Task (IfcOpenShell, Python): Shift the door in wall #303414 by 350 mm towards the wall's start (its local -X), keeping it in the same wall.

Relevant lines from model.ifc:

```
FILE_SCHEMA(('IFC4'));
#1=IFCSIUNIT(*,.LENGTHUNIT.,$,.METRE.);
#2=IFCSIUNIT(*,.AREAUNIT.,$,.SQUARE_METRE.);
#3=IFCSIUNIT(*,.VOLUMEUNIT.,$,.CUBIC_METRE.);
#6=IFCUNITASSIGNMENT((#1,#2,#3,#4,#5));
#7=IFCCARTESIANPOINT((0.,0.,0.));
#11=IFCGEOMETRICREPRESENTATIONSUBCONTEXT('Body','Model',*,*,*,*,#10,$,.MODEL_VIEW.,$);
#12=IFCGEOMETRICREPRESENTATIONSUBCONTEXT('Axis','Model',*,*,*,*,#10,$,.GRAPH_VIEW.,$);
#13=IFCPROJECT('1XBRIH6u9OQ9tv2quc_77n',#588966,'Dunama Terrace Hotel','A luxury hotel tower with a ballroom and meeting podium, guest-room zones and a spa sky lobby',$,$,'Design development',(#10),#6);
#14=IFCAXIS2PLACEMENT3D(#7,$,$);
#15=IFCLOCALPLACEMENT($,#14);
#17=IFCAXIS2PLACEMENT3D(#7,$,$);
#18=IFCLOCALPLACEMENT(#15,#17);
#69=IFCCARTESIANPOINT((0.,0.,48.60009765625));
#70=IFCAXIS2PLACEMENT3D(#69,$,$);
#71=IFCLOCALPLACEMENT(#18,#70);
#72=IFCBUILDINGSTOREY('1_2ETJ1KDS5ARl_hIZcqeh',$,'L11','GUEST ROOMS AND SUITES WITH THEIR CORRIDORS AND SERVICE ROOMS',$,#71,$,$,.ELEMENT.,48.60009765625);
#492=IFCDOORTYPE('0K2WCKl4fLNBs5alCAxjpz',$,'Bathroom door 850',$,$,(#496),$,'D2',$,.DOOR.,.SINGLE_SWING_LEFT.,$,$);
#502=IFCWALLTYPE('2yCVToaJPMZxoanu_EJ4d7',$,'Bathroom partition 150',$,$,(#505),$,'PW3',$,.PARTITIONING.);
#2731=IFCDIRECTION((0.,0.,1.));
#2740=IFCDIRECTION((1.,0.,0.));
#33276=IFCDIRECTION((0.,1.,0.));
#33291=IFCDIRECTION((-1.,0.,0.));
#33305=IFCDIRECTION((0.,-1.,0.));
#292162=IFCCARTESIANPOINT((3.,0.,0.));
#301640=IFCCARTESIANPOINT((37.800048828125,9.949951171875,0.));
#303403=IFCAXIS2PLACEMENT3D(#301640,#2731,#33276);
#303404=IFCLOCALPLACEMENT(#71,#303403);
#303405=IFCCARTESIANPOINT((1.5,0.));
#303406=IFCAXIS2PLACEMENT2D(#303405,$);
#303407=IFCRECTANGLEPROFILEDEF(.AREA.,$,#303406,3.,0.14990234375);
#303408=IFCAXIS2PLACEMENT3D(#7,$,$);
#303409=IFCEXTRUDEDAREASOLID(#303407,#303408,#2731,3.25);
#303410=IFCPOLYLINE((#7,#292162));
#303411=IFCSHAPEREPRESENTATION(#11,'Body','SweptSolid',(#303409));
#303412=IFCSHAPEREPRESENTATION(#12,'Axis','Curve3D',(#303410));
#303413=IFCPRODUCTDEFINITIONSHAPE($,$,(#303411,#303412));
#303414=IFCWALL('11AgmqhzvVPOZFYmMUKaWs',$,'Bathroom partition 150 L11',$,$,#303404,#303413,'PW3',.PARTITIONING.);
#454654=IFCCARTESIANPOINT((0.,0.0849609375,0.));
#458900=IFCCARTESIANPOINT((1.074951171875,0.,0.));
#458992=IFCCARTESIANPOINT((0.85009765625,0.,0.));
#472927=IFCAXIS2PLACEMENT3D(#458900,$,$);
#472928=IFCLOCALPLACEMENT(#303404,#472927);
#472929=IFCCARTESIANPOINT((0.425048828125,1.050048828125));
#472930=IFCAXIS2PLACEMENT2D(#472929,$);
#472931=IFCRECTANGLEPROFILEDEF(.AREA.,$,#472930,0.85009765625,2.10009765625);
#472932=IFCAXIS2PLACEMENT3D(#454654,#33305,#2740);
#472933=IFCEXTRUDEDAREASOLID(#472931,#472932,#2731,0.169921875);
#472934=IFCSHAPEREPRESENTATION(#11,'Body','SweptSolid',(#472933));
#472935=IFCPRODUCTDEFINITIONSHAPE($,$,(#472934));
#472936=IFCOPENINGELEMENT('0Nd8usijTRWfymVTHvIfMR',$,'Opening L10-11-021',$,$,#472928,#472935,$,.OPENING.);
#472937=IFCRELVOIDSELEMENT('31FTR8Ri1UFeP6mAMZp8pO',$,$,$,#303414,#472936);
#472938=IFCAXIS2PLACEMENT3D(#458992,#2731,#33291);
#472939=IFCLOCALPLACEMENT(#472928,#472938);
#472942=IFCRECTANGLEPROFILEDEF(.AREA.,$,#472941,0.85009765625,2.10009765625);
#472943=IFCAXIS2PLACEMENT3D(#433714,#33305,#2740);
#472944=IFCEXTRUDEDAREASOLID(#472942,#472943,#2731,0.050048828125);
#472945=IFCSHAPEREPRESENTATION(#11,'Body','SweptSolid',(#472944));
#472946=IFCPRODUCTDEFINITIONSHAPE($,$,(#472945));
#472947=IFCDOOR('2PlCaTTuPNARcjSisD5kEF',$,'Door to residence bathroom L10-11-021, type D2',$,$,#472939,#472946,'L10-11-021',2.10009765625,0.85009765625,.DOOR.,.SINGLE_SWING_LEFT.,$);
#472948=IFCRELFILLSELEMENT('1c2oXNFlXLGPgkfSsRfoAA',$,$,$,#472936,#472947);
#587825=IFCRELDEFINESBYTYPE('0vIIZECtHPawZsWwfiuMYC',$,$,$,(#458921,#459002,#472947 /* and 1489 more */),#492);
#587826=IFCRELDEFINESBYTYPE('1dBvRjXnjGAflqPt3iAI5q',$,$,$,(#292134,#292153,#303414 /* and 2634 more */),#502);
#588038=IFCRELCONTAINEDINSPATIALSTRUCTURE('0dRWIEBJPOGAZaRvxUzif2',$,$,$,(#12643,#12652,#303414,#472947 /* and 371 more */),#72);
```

```python
import ifcopenshell
import ifcopenshell.api.geometry
import ifcopenshell.util.placement
import ifcopenshell.util.unit

model = ifcopenshell.open("model.ifc")
unit_scale = ifcopenshell.util.unit.calculate_unit_scale(model)

door = model.by_guid("2PlCaTTuPNARcjSisD5kEF")
opening = door.FillsVoids[0].RelatingOpeningElement
wall = opening.VoidsElements[0].RelatingBuildingElement

wall_matrix = ifcopenshell.util.placement.get_local_placement(wall.ObjectPlacement)
shift = wall_matrix[:3, 0] * -0.35 / unit_scale
before = ifcopenshell.util.placement.get_local_placement(door.ObjectPlacement)[:3, 3].copy()

# The door is placed relative to its opening, so it follows when the opening moves.
matrix = ifcopenshell.util.placement.get_local_placement(opening.ObjectPlacement)
matrix[:3, 3] += shift
ifcopenshell.api.geometry.edit_object_placement(
    model, product=opening, matrix=matrix, is_si=False, should_transform_children=True
)

after = ifcopenshell.util.placement.get_local_placement(door.ObjectPlacement)[:3, 3]
print("door moved by", (after - before).round(3) + 0.0)

model.write("model_updated.ifc")
```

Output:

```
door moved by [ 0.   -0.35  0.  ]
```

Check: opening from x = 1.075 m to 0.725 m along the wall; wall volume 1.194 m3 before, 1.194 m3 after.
